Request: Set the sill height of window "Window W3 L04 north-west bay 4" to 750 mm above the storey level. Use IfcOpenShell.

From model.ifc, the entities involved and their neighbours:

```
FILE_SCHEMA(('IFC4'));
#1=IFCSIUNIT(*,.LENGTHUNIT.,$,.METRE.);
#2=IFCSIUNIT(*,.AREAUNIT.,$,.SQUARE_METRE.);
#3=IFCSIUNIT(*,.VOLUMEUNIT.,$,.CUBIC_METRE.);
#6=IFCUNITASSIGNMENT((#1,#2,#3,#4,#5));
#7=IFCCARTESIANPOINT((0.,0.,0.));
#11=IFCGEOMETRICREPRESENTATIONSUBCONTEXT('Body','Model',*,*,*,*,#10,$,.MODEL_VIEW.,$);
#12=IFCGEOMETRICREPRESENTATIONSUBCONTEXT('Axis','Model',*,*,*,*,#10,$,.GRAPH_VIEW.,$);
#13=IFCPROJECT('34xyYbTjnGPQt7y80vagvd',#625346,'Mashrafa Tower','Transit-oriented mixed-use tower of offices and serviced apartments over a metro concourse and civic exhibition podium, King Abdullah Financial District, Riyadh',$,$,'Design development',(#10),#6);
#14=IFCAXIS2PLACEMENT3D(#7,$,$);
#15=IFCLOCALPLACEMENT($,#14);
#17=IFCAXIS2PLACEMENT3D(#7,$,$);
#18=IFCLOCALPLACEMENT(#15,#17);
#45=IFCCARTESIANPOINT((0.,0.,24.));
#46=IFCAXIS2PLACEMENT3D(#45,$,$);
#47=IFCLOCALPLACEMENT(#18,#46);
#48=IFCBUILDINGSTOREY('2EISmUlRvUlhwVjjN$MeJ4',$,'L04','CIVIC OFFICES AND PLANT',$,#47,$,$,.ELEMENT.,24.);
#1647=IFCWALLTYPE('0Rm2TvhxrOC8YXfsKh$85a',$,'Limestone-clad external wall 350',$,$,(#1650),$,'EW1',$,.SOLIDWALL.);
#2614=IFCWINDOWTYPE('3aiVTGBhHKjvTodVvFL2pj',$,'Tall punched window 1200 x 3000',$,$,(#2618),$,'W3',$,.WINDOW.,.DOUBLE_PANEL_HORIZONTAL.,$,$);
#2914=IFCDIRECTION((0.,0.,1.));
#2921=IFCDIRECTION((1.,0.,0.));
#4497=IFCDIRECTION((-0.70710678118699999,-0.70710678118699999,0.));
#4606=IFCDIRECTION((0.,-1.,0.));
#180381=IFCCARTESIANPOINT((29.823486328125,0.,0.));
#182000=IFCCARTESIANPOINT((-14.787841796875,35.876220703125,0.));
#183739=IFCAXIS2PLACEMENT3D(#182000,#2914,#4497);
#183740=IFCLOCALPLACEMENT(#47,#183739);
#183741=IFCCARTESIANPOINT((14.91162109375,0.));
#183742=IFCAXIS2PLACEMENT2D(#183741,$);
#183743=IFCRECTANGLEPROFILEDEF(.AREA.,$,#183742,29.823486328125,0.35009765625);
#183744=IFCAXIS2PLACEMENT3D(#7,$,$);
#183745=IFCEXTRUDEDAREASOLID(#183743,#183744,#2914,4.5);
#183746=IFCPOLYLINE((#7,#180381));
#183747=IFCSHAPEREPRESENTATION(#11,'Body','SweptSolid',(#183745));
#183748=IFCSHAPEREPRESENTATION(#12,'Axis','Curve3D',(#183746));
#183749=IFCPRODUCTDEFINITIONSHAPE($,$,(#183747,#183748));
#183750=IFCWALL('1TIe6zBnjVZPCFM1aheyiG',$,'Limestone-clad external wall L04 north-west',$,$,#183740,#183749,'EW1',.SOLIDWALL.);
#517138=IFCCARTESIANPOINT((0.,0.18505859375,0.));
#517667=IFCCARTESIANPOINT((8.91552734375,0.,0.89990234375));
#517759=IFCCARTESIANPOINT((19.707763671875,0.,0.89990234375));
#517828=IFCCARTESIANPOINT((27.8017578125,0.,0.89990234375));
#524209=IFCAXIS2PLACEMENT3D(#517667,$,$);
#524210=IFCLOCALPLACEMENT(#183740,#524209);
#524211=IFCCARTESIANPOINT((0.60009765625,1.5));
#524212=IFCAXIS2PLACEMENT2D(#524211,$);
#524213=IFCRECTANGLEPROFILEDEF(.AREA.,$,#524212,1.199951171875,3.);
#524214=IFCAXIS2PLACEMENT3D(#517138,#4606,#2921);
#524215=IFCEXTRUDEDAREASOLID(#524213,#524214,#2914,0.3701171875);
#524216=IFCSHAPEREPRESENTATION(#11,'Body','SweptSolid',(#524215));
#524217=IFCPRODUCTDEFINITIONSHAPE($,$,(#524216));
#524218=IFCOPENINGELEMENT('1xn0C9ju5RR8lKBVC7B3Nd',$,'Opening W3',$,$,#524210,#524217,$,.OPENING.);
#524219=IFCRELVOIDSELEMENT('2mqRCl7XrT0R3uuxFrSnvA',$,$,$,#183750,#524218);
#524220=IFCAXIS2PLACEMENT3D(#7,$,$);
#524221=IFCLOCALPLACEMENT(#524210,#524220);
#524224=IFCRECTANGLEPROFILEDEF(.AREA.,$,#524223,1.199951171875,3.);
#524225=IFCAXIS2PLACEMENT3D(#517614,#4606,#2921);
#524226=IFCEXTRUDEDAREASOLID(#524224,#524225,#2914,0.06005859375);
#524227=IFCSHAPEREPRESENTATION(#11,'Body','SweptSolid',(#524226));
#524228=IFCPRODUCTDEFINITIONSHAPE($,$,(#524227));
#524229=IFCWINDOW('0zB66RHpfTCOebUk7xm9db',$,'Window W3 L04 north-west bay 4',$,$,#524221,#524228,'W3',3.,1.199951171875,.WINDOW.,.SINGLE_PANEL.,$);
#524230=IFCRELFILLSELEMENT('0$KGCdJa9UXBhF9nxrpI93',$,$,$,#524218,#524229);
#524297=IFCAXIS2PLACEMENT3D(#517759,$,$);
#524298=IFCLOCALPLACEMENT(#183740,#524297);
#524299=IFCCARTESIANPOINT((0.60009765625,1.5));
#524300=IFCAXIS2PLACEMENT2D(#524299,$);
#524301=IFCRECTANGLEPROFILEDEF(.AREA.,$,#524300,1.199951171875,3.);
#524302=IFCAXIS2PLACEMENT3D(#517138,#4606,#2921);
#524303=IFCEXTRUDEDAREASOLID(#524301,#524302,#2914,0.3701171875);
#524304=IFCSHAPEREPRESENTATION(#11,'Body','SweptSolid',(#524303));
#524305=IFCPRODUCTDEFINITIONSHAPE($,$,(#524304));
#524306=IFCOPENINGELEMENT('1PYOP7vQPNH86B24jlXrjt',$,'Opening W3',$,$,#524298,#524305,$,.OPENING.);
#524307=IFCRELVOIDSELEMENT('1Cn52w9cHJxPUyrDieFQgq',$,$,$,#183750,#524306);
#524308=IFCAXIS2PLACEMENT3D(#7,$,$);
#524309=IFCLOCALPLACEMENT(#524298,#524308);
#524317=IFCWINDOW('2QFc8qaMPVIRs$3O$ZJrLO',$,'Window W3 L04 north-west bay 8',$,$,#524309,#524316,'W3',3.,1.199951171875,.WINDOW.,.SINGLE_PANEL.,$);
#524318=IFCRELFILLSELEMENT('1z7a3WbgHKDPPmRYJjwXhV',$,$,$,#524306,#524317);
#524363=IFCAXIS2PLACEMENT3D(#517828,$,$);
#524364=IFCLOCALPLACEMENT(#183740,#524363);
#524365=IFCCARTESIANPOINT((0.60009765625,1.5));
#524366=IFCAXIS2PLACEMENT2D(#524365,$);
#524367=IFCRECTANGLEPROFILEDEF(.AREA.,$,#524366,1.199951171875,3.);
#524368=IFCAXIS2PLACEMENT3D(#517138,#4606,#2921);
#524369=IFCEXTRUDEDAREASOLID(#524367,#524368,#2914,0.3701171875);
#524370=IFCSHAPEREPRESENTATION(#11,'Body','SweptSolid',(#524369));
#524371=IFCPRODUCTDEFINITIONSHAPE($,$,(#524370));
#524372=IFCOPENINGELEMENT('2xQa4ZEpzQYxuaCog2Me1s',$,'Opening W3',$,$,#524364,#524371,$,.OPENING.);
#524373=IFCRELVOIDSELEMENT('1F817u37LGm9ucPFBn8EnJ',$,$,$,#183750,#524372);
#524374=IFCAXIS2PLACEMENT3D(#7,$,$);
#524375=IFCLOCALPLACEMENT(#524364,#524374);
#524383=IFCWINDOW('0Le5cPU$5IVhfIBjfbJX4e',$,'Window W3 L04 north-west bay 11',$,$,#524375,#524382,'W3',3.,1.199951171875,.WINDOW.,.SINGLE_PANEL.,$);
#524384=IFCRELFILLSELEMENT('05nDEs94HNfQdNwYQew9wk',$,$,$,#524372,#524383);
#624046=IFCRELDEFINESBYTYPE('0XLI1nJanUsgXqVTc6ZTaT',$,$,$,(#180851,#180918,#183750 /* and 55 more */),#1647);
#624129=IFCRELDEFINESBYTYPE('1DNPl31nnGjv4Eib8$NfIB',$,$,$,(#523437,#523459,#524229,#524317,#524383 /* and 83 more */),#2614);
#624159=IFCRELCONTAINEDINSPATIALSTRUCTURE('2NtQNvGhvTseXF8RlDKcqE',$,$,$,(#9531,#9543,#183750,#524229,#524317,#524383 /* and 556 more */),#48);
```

```python
import numpy as np
import ifcopenshell
import ifcopenshell.api.geometry
import ifcopenshell.geom
import ifcopenshell.util.element
import ifcopenshell.util.placement
import ifcopenshell.util.shape
import ifcopenshell.util.unit

model = ifcopenshell.open("model.ifc")
unit_scale = ifcopenshell.util.unit.calculate_unit_scale(model)

window = model.by_guid("0zB66RHpfTCOebUk7xm9db")
opening = window.FillsVoids[0].RelatingOpeningElement
storey = ifcopenshell.util.element.get_container(window, ifc_class="IfcBuildingStorey")
level = ifcopenshell.util.placement.get_local_placement(storey.ObjectPlacement)[2, 3]

# The opening's origin need not be at the sill, so measure its lowest point.
shape = ifcopenshell.geom.create_shape(ifcopenshell.geom.settings(), opening)
bottom = ifcopenshell.util.shape.get_shape_bottom_elevation(shape, shape.geometry) / unit_scale
dz = level + 0.75 / unit_scale - bottom

shift = np.array([0.0, 0.0, dz])
# The window is placed relative to its opening, so it follows when the opening moves.
matrix = ifcopenshell.util.placement.get_local_placement(opening.ObjectPlacement)
matrix[:3, 3] += shift
ifcopenshell.api.geometry.edit_object_placement(
    model, product=opening, matrix=matrix, is_si=False, should_transform_children=True
)

print(f"moved by {dz * unit_scale:+.3f} m")

model.write("model_rev.ifc")
```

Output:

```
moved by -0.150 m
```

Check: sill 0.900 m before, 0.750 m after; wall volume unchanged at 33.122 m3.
